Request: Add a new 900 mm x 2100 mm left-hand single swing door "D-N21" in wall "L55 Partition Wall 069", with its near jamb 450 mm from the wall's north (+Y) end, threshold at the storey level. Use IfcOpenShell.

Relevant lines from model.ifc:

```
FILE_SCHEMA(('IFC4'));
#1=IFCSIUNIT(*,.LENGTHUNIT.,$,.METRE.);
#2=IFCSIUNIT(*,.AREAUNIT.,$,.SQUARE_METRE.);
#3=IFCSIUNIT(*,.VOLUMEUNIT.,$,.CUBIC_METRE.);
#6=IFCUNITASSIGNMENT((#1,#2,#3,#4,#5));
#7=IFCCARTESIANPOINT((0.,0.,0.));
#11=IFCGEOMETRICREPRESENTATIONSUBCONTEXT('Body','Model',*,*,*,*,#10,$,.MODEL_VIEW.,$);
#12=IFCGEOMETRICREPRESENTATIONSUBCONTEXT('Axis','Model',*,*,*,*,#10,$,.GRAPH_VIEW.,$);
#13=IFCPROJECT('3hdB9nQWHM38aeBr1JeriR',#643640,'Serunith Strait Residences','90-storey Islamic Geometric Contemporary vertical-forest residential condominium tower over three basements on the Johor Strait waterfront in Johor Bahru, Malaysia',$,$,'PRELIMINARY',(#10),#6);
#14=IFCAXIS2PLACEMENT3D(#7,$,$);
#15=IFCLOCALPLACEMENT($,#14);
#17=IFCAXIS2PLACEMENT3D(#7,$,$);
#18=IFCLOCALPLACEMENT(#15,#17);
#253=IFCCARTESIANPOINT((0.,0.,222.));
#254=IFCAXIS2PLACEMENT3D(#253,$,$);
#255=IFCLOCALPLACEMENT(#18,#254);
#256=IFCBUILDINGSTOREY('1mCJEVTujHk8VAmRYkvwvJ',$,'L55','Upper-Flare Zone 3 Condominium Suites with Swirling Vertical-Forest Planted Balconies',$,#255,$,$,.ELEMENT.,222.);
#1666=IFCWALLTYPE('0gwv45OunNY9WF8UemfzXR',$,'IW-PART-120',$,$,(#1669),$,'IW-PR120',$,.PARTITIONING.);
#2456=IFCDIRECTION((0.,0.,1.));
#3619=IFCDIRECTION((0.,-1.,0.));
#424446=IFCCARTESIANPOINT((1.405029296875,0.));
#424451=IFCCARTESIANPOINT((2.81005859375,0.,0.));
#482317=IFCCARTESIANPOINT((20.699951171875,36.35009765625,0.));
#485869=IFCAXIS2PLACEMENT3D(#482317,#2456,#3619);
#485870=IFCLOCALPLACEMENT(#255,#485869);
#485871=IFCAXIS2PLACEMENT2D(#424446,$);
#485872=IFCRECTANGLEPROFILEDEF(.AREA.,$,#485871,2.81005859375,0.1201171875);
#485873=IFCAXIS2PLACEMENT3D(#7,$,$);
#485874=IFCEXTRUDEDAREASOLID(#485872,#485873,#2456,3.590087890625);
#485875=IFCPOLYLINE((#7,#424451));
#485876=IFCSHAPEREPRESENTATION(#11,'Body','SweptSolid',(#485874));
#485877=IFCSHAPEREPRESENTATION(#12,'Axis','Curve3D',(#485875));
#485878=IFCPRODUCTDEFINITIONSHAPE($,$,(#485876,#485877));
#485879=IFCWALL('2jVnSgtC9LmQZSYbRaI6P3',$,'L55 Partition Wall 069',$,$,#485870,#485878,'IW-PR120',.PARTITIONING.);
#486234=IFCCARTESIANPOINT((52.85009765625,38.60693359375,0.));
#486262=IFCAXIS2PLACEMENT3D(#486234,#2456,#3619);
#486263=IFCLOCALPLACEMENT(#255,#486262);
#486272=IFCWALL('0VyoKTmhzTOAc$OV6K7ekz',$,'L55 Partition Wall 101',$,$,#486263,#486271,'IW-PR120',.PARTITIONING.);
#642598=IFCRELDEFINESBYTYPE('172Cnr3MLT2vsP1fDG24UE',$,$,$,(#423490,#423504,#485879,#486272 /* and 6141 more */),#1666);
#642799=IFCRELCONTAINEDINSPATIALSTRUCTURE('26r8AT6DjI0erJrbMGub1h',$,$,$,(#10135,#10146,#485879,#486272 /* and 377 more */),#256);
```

```python
import numpy as np
import ifcopenshell
import ifcopenshell.api.feature
import ifcopenshell.api.geometry
import ifcopenshell.api.root
import ifcopenshell.api.spatial
import ifcopenshell.geom
import ifcopenshell.util.element
import ifcopenshell.util.placement
import ifcopenshell.util.representation
import ifcopenshell.util.shape
import ifcopenshell.util.unit

model = ifcopenshell.open("model.ifc")
unit_scale = ifcopenshell.util.unit.calculate_unit_scale(model)
settings = ifcopenshell.geom.settings()


def volume(element):
    """Net volume in cubic metres, openings subtracted."""
    shape = ifcopenshell.geom.create_shape(settings, element)
    return ifcopenshell.util.shape.get_volume(shape.geometry)


wall = model.by_guid("2jVnSgtC9LmQZSYbRaI6P3")
storey = ifcopenshell.util.element.get_container(wall, ifc_class="IfcBuildingStorey")
context = ifcopenshell.util.representation.get_context(model, "Model", "Body", "MODEL_VIEW")
before = volume(wall)

width, height, from_end, sill = 0.9, 2.1, 0.45, 0.0  # metres

# The wall runs along its own X axis, and the end named is its -X end.
wall_shape = ifcopenshell.geom.create_shape(settings, wall)
x, y, z = ifcopenshell.util.shape.get_vertices(wall_shape.geometry).T
start = x.min() + from_end
face, thickness = float(y.min()), float(y.max() - y.min())
wall_matrix = ifcopenshell.util.placement.get_local_placement(wall.ObjectPlacement)
level = ifcopenshell.util.placement.get_local_placement(storey.ObjectPlacement)[2, 3]


def in_wall(x, y):
    """Placement at x, y metres in the wall's axes, at sill height."""
    matrix = wall_matrix.copy()
    matrix[:, 3] = wall_matrix @ np.array([x / unit_scale, y / unit_scale, 0.0, 1.0])
    matrix[2, 3] = level + sill / unit_scale
    return matrix


# Opening: a box that overshoots both wall faces by 50 mm.
opening = ifcopenshell.api.root.create_entity(model, ifc_class="IfcOpeningElement", predefined_type="OPENING")
box = ifcopenshell.api.geometry.add_wall_representation(
    model, context=context, length=width, height=height, thickness=thickness + 0.1
)
ifcopenshell.api.geometry.assign_representation(model, product=opening, representation=box)
ifcopenshell.api.geometry.edit_object_placement(model, product=opening, matrix=in_wall(start, face - 0.05), is_si=False)
ifcopenshell.api.feature.add_feature(model, feature=opening, element=wall)

door = ifcopenshell.api.root.create_entity(model, ifc_class="IfcDoor", name="D-N21", predefined_type="DOOR")
door.OverallWidth, door.OverallHeight = width / unit_scale, height / unit_scale
door.OperationType = "SINGLE_SWING_LEFT"
body = ifcopenshell.api.geometry.add_door_representation(
    model,
    context=context,
    overall_width=door.OverallWidth,
    overall_height=door.OverallHeight,
    operation_type="SINGLE_SWING_LEFT",
    lining_properties={"LiningDepth": thickness / unit_scale, "ThresholdDepth": thickness / unit_scale},
)
ifcopenshell.api.geometry.assign_representation(model, product=door, representation=body)
ifcopenshell.api.spatial.assign_container(model, products=[door], relating_structure=storey)
ifcopenshell.api.feature.add_filling(model, opening=opening, element=door)

# The lining spans the wall, so the door starts at the wall face.
ifcopenshell.api.geometry.edit_object_placement(model, product=door, matrix=in_wall(start, face), is_si=False)

after = volume(wall)

print(f"wall volume {before:.3f} -> {after:.3f} m3")

model.write("model_v2.ifc")
```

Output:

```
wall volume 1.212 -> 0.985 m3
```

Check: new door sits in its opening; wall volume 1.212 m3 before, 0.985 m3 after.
